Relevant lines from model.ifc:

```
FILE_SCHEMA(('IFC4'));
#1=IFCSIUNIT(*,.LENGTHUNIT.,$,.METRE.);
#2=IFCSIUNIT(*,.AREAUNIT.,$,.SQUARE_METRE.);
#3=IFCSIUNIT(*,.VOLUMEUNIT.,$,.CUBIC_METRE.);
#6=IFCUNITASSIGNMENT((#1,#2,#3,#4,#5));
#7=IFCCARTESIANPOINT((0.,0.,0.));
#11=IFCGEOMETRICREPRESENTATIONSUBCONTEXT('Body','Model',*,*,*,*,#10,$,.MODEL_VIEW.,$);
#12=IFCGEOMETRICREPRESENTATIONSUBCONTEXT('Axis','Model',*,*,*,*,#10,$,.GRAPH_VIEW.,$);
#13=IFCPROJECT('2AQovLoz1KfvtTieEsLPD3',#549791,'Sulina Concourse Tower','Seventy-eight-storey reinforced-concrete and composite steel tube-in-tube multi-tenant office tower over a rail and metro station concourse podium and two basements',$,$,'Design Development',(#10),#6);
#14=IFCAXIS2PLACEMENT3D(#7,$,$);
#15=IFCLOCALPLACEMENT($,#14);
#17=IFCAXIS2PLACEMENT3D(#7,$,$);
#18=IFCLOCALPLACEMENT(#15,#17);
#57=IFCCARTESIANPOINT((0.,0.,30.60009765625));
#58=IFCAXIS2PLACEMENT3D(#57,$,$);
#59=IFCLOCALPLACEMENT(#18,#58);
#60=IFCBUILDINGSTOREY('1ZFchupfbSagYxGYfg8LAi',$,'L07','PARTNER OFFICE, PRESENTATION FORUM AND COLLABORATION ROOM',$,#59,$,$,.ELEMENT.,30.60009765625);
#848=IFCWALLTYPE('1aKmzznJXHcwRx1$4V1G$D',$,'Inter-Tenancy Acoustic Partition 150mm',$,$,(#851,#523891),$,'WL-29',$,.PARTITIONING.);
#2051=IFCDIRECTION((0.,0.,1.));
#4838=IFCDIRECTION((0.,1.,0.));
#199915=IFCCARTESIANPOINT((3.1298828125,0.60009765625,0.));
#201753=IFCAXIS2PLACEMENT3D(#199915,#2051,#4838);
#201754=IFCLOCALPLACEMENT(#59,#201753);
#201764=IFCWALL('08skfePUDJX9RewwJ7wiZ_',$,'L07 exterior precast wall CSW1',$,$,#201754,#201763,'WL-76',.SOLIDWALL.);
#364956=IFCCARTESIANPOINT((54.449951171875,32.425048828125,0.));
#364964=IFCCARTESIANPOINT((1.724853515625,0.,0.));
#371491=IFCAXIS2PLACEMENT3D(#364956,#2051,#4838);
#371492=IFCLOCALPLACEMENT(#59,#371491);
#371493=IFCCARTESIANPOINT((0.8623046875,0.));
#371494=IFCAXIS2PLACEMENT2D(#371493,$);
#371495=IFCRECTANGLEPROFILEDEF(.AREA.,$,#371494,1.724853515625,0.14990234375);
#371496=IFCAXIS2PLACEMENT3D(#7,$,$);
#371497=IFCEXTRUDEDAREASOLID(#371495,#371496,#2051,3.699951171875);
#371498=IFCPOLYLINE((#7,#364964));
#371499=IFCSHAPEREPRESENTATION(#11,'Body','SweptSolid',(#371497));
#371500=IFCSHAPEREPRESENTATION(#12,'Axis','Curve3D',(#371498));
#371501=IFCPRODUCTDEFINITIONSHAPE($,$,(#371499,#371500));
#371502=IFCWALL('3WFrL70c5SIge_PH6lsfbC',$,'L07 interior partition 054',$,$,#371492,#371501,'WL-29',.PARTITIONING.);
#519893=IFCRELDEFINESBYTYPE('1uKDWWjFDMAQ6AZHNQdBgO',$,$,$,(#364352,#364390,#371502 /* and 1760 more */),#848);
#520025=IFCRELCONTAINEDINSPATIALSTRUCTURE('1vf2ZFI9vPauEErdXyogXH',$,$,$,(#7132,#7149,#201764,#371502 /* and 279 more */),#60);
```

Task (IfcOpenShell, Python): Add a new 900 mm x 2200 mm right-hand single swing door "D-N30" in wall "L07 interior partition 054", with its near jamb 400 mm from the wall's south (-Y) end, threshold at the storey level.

```python
import numpy as np
import ifcopenshell
import ifcopenshell.api.feature
import ifcopenshell.api.geometry
import ifcopenshell.api.root
import ifcopenshell.api.spatial
import ifcopenshell.geom
import ifcopenshell.util.element
import ifcopenshell.util.placement
import ifcopenshell.util.representation
import ifcopenshell.util.shape
import ifcopenshell.util.unit

model = ifcopenshell.open("model.ifc")
unit_scale = ifcopenshell.util.unit.calculate_unit_scale(model)
settings = ifcopenshell.geom.settings()


def volume(element):
    """Net volume in cubic metres, openings subtracted."""
    shape = ifcopenshell.geom.create_shape(settings, element)
    return ifcopenshell.util.shape.get_volume(shape.geometry)


wall = model.by_guid("3WFrL70c5SIge_PH6lsfbC")
storey = ifcopenshell.util.element.get_container(wall, ifc_class="IfcBuildingStorey")
context = ifcopenshell.util.representation.get_context(model, "Model", "Body", "MODEL_VIEW")
before = volume(wall)

width, height, from_end, sill = 0.9, 2.2, 0.4, 0.0  # metres

# The wall runs along its own X axis, and the end named is its -X end.
wall_shape = ifcopenshell.geom.create_shape(settings, wall)
x, y, z = ifcopenshell.util.shape.get_vertices(wall_shape.geometry).T
start = x.min() + from_end
face, thickness = float(y.min()), float(y.max() - y.min())
wall_matrix = ifcopenshell.util.placement.get_local_placement(wall.ObjectPlacement)
level = ifcopenshell.util.placement.get_local_placement(storey.ObjectPlacement)[2, 3]


def in_wall(x, y):
    """Placement at x, y metres in the wall's axes, at sill height."""
    matrix = wall_matrix.copy()
    matrix[:, 3] = wall_matrix @ np.array([x / unit_scale, y / unit_scale, 0.0, 1.0])
    matrix[2, 3] = level + sill / unit_scale
    return matrix


# Opening: a box that overshoots both wall faces by 50 mm.
opening = ifcopenshell.api.root.create_entity(model, ifc_class="IfcOpeningElement", predefined_type="OPENING")
box = ifcopenshell.api.geometry.add_wall_representation(
    model, context=context, length=width, height=height, thickness=thickness + 0.1
)
ifcopenshell.api.geometry.assign_representation(model, product=opening, representation=box)
ifcopenshell.api.geometry.edit_object_placement(model, product=opening, matrix=in_wall(start, face - 0.05), is_si=False)
ifcopenshell.api.feature.add_feature(model, feature=opening, element=wall)

door = ifcopenshell.api.root.create_entity(model, ifc_class="IfcDoor", name="D-N30", predefined_type="DOOR")
door.OverallWidth, door.OverallHeight = width / unit_scale, height / unit_scale
door.OperationType = "SINGLE_SWING_RIGHT"
body = ifcopenshell.api.geometry.add_door_representation(
    model,
    context=context,
    overall_width=door.OverallWidth,
    overall_height=door.OverallHeight,
    operation_type="SINGLE_SWING_RIGHT",
    lining_properties={"LiningDepth": thickness / unit_scale, "ThresholdDepth": thickness / unit_scale},
)
ifcopenshell.api.geometry.assign_representation(model, product=door, representation=body)
ifcopenshell.api.spatial.assign_container(model, products=[door], relating_structure=storey)
ifcopenshell.api.feature.add_filling(model, opening=opening, element=door)

# The lining spans the wall, so the door starts at the wall face.
ifcopenshell.api.geometry.edit_object_placement(model, product=door, matrix=in_wall(start, face), is_si=False)

after = volume(wall)

print(f"wall volume {before:.3f} -> {after:.3f} m3")

model.write("model-out.ifc")
```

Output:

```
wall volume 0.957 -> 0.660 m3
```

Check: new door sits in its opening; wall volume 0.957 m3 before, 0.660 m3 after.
